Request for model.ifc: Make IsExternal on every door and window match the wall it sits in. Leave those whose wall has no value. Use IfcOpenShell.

First a look at what the model holds.

```python
import ifcopenshell
import ifcopenshell.util.element

model = ifcopenshell.open("model.ifc")
print(model.schema)
seen = {}
for e in model.by_type("IfcDoor") + model.by_type("IfcWindow"):
    if not e.FillsVoids:
        continue
    host = e.FillsVoids[0].RelatingOpeningElement.VoidsElements[0].RelatingBuildingElement
    own = ifcopenshell.util.element.get_pset(e, f"Pset_{e.is_a()[3:].removesuffix('StandardCase')}Common", "IsExternal")
    wall = ifcopenshell.util.element.get_pset(host, "Pset_WallCommon", "IsExternal")
    seen[e.is_a(), own, wall] = seen.get((e.is_a(), own, wall), 0) + 1
for (cls, own, wall), count in sorted(seen.items(), key=str):
    print(count, cls, "IsExternal:", own, "| host wall:", wall)
```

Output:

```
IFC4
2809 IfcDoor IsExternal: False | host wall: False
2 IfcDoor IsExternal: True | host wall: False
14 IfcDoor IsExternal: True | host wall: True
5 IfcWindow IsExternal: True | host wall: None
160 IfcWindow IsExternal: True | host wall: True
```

```python
import ifcopenshell
import ifcopenshell.api.pset
import ifcopenshell.util.element

model = ifcopenshell.open("model.ifc")

count = 0
for ifc_class, pset_name in (("IfcDoor", "Pset_DoorCommon"), ("IfcWindow", "Pset_WindowCommon")):
    for e in model.by_type(ifc_class):
        if not e.FillsVoids:
            continue
        host = e.FillsVoids[0].RelatingOpeningElement.VoidsElements[0].RelatingBuildingElement
        external = ifcopenshell.util.element.get_pset(host, "Pset_WallCommon", "IsExternal")
        if external is None or ifcopenshell.util.element.get_pset(e, pset_name, "IsExternal") == external:
            continue
        pset = ifcopenshell.api.pset.add_pset(model, product=e, name=pset_name)
        ifcopenshell.api.pset.edit_pset(model, pset=pset, properties={"IsExternal": external})
        count += 1

print(count, "updated")

model.write("model_updated.ifc")
```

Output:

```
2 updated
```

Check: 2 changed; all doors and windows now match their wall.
